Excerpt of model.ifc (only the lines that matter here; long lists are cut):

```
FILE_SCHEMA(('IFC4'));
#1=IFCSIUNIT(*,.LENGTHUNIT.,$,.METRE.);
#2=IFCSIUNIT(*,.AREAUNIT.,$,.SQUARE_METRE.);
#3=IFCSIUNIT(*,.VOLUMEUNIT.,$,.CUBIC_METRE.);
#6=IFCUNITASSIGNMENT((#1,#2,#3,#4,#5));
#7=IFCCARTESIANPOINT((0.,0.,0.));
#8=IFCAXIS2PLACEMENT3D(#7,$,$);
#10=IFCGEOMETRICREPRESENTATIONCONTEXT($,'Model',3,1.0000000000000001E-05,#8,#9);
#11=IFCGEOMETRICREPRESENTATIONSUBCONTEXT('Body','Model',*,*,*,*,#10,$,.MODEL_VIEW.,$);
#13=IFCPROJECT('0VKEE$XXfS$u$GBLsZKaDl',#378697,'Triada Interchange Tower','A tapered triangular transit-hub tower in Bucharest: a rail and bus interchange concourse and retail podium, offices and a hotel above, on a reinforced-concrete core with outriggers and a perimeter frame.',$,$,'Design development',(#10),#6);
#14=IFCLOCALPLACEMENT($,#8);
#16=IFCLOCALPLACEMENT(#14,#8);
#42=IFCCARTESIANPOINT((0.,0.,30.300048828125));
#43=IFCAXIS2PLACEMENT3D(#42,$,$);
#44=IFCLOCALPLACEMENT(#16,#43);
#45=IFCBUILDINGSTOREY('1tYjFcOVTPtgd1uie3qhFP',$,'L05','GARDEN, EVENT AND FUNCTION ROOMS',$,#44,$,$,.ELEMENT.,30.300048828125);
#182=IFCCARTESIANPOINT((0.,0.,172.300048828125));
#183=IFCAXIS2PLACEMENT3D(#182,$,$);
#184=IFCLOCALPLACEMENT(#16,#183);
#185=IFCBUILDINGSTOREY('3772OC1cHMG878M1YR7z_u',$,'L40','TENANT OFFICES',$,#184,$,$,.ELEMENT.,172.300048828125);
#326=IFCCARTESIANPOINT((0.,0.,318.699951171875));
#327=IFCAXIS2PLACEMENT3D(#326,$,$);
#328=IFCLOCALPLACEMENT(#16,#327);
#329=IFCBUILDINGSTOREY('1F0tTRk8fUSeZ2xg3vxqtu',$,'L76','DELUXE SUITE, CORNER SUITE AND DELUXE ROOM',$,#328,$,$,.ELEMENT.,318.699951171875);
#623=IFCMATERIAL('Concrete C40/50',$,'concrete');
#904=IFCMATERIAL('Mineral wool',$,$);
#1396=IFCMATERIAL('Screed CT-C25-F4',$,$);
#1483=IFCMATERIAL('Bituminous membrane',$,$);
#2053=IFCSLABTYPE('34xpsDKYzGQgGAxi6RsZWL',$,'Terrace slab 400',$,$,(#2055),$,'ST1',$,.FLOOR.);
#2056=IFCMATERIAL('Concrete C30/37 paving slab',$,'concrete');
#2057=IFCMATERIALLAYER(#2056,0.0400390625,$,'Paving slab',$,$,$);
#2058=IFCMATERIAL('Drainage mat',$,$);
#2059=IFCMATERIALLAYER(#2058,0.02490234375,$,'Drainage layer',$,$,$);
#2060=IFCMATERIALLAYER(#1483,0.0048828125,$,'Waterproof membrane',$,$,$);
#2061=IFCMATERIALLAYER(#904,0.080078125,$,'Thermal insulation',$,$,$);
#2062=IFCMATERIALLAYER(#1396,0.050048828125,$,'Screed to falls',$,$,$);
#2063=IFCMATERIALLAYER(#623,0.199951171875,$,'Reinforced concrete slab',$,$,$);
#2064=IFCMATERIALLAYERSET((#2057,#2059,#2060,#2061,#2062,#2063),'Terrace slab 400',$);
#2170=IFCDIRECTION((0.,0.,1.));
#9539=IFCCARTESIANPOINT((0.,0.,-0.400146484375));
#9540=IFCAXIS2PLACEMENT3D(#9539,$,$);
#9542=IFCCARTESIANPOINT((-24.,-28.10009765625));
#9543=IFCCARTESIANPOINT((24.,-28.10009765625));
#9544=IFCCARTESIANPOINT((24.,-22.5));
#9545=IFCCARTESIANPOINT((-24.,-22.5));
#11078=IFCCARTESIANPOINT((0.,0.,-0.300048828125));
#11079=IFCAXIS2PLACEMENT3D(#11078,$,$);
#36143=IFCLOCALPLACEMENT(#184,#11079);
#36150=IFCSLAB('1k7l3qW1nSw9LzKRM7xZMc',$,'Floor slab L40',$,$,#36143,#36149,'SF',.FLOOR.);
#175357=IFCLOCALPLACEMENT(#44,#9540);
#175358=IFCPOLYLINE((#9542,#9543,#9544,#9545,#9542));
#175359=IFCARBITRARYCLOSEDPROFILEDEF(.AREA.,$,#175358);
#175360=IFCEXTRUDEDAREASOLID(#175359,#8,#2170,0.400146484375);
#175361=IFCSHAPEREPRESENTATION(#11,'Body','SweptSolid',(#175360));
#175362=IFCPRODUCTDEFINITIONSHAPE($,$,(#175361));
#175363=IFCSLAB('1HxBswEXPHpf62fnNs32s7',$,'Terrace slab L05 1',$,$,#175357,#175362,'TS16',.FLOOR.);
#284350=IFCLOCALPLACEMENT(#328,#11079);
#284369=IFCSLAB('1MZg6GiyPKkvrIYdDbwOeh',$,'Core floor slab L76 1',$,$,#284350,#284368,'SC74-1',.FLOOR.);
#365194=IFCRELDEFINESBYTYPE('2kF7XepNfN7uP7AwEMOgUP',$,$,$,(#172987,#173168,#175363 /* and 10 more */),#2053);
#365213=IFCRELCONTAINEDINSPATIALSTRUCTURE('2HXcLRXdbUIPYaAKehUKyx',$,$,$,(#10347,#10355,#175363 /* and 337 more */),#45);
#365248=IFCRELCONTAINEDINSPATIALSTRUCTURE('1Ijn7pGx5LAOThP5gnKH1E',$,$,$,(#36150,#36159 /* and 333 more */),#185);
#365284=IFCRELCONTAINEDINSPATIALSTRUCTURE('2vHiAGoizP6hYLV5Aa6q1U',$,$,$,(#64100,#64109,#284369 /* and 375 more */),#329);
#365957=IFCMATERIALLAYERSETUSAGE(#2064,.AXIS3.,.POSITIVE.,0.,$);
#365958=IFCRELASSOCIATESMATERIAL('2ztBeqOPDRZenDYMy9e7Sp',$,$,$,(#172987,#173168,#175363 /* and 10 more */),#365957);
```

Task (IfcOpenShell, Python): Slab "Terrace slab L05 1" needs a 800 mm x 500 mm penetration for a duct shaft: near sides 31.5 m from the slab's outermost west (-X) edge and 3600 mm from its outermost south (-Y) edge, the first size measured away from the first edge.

```python
import numpy as np
import ifcopenshell
import ifcopenshell.api.feature
import ifcopenshell.api.geometry
import ifcopenshell.api.root
import ifcopenshell.geom
import ifcopenshell.util.placement
import ifcopenshell.util.representation
import ifcopenshell.util.shape
import ifcopenshell.util.unit

model = ifcopenshell.open("model.ifc")
unit_scale = ifcopenshell.util.unit.calculate_unit_scale(model)
settings = ifcopenshell.geom.settings()


def volume(element):
    """Net volume in cubic metres, openings subtracted."""
    shape = ifcopenshell.geom.create_shape(settings, element)
    return ifcopenshell.util.shape.get_volume(shape.geometry)


slab = model.by_guid("1HxBswEXPHpf62fnNs32s7")
before = volume(slab)

# Extent in the slab's own axes, in metres. The edges named are its -X and -Y sides.
slab_shape = ifcopenshell.geom.create_shape(settings, slab)
vertices = ifcopenshell.util.shape.get_vertices(slab_shape.geometry)
x_min, y_min, bottom = vertices.min(axis=0)
top = vertices[:, 2].max()

opening = ifcopenshell.api.root.create_entity(model, ifc_class="IfcOpeningElement", name="Duct shaft opening", predefined_type="OPENING")
context = ifcopenshell.util.representation.get_context(model, "Model", "Body", "MODEL_VIEW")
width, depth = 0.8, 0.5
outline = [(0.0, 0.0), (width, 0.0), (width, depth), (0.0, depth), (0.0, 0.0)]
# Overshoot both faces by 50 mm so the cut is clean.
shape = ifcopenshell.api.geometry.add_slab_representation(
    model, context=context, depth=top - bottom + 0.1, polyline=outline
)
ifcopenshell.api.geometry.assign_representation(model, product=opening, representation=shape)

matrix = ifcopenshell.util.placement.get_local_placement(slab.ObjectPlacement)
matrix[:, 3] = matrix @ np.append(np.array([x_min + 31.5, y_min + 3.6, bottom - 0.05]) / unit_scale, 1.0)
ifcopenshell.api.geometry.edit_object_placement(model, product=opening, matrix=matrix, is_si=False)
ifcopenshell.api.feature.add_feature(model, feature=opening, element=slab)

after = volume(slab)

print(f"slab volume {before:.3f} -> {after:.3f} m3")

model.write("model_updated.ifc")
```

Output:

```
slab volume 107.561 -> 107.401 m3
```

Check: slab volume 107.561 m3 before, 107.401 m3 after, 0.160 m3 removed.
